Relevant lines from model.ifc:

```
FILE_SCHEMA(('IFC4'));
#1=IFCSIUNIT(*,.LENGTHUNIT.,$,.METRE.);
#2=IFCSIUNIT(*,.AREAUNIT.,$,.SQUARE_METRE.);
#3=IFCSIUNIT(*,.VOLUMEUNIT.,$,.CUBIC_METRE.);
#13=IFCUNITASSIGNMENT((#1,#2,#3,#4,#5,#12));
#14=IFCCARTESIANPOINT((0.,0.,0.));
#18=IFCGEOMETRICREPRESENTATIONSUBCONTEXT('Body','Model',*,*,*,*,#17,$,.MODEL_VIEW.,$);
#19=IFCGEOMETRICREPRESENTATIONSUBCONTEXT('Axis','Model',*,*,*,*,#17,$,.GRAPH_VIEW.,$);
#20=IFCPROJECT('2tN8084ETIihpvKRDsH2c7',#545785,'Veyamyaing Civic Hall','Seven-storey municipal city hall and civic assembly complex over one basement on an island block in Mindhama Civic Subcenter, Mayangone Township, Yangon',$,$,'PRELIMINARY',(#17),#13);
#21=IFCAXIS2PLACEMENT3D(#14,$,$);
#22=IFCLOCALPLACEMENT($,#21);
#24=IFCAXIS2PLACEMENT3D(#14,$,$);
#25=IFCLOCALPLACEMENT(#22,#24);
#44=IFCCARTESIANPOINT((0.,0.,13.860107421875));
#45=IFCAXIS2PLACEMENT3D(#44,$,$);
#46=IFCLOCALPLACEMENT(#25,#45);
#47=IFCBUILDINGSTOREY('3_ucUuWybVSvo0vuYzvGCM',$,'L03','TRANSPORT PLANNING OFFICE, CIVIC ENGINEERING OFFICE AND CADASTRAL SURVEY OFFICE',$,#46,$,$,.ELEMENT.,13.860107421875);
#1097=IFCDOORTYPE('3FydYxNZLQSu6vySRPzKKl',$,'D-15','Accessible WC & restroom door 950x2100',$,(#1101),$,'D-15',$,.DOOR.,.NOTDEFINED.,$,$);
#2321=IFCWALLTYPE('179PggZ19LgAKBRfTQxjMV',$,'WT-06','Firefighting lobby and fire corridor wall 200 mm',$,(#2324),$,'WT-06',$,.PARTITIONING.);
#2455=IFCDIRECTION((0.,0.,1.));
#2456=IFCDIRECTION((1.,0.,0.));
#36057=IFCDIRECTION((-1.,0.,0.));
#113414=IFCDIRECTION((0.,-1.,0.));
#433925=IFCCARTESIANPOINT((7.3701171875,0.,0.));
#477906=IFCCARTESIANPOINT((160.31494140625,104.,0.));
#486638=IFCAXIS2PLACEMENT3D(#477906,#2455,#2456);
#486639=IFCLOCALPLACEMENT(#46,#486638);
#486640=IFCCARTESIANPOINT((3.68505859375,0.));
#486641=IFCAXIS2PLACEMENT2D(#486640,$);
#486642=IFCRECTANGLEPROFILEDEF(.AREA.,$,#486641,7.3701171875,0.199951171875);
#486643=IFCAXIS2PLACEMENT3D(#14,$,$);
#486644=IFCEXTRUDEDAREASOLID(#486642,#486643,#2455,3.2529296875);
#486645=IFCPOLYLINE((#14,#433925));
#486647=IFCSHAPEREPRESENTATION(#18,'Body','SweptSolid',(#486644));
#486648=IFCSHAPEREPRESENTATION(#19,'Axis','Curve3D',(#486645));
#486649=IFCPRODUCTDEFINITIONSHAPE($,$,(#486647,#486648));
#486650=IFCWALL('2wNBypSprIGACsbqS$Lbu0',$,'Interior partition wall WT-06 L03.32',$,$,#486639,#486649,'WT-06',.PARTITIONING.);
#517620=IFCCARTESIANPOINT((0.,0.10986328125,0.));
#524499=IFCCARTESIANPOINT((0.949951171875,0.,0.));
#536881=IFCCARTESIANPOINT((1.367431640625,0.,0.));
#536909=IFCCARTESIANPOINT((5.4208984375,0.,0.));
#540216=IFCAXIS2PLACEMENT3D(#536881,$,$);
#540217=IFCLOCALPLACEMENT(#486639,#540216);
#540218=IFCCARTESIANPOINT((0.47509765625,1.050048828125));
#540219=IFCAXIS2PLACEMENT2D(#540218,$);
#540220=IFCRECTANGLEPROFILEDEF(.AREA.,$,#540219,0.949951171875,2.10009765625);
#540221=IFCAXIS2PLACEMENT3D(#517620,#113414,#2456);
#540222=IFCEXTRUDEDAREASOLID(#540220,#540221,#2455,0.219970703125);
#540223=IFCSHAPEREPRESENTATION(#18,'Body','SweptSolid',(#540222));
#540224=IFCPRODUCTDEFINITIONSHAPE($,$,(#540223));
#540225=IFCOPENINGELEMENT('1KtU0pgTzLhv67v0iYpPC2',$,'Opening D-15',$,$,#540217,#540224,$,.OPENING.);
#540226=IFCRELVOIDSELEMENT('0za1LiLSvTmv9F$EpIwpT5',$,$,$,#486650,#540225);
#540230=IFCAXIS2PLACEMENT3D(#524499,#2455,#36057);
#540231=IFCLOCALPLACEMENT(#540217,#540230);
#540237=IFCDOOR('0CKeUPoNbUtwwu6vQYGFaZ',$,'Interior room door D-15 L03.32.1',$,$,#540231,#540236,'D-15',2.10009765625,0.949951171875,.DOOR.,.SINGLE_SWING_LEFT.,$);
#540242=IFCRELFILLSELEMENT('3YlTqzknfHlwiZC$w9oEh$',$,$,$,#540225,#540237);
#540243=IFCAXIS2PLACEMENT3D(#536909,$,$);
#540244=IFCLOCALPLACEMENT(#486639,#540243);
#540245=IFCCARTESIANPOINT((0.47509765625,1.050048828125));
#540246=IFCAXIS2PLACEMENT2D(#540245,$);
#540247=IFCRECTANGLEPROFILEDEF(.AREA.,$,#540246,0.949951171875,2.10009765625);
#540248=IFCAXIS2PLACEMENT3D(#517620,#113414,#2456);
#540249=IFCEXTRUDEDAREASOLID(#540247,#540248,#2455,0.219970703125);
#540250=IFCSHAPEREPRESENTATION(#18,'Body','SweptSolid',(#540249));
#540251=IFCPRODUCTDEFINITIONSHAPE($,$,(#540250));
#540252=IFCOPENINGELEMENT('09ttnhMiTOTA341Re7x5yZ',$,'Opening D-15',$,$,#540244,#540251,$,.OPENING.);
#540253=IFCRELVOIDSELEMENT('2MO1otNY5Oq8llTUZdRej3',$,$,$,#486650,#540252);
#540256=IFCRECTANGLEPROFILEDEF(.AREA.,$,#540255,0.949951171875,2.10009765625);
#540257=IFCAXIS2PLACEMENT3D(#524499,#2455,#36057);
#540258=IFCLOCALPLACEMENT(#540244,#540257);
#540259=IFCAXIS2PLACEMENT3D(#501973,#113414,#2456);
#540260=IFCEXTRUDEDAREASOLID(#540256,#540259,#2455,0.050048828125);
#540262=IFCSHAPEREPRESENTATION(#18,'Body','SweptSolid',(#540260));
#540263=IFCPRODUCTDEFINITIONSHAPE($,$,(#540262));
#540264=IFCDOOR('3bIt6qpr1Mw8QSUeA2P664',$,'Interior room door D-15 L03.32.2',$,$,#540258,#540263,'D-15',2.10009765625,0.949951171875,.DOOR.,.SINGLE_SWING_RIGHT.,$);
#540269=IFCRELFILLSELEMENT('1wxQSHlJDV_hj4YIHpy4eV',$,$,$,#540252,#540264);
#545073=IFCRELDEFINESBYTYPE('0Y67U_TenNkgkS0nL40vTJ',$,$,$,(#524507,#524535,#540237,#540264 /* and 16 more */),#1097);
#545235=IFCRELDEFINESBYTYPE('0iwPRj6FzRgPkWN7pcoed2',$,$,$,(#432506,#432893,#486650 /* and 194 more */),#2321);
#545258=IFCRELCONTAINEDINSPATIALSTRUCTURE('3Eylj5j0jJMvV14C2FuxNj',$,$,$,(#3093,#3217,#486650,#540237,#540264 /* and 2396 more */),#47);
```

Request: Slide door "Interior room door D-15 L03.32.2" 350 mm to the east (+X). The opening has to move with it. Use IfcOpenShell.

```python
import ifcopenshell
import ifcopenshell.api.geometry
import ifcopenshell.util.placement

model = ifcopenshell.open("model.ifc")

door = model.by_guid("3bIt6qpr1Mw8QSUeA2P664")
opening = door.FillsVoids[0].RelatingOpeningElement
wall = opening.VoidsElements[0].RelatingBuildingElement

wall_matrix = ifcopenshell.util.placement.get_local_placement(wall.ObjectPlacement)
shift = wall_matrix[:3, 0] * 0.35
before = ifcopenshell.util.placement.get_local_placement(door.ObjectPlacement)[:3, 3].copy()

# The door is placed relative to its opening, so it follows when the opening moves.
matrix = ifcopenshell.util.placement.get_local_placement(opening.ObjectPlacement)
matrix[:3, 3] += shift
ifcopenshell.api.geometry.edit_object_placement(
    model, product=opening, matrix=matrix, is_si=False, should_transform_children=True
)

after = ifcopenshell.util.placement.get_local_placement(door.ObjectPlacement)[:3, 3]
print("door moved by", (after - before).round(3) + 0.0)

model.write("model_updated.ifc")
```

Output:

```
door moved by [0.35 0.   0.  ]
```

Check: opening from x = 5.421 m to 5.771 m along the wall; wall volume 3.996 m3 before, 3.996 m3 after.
